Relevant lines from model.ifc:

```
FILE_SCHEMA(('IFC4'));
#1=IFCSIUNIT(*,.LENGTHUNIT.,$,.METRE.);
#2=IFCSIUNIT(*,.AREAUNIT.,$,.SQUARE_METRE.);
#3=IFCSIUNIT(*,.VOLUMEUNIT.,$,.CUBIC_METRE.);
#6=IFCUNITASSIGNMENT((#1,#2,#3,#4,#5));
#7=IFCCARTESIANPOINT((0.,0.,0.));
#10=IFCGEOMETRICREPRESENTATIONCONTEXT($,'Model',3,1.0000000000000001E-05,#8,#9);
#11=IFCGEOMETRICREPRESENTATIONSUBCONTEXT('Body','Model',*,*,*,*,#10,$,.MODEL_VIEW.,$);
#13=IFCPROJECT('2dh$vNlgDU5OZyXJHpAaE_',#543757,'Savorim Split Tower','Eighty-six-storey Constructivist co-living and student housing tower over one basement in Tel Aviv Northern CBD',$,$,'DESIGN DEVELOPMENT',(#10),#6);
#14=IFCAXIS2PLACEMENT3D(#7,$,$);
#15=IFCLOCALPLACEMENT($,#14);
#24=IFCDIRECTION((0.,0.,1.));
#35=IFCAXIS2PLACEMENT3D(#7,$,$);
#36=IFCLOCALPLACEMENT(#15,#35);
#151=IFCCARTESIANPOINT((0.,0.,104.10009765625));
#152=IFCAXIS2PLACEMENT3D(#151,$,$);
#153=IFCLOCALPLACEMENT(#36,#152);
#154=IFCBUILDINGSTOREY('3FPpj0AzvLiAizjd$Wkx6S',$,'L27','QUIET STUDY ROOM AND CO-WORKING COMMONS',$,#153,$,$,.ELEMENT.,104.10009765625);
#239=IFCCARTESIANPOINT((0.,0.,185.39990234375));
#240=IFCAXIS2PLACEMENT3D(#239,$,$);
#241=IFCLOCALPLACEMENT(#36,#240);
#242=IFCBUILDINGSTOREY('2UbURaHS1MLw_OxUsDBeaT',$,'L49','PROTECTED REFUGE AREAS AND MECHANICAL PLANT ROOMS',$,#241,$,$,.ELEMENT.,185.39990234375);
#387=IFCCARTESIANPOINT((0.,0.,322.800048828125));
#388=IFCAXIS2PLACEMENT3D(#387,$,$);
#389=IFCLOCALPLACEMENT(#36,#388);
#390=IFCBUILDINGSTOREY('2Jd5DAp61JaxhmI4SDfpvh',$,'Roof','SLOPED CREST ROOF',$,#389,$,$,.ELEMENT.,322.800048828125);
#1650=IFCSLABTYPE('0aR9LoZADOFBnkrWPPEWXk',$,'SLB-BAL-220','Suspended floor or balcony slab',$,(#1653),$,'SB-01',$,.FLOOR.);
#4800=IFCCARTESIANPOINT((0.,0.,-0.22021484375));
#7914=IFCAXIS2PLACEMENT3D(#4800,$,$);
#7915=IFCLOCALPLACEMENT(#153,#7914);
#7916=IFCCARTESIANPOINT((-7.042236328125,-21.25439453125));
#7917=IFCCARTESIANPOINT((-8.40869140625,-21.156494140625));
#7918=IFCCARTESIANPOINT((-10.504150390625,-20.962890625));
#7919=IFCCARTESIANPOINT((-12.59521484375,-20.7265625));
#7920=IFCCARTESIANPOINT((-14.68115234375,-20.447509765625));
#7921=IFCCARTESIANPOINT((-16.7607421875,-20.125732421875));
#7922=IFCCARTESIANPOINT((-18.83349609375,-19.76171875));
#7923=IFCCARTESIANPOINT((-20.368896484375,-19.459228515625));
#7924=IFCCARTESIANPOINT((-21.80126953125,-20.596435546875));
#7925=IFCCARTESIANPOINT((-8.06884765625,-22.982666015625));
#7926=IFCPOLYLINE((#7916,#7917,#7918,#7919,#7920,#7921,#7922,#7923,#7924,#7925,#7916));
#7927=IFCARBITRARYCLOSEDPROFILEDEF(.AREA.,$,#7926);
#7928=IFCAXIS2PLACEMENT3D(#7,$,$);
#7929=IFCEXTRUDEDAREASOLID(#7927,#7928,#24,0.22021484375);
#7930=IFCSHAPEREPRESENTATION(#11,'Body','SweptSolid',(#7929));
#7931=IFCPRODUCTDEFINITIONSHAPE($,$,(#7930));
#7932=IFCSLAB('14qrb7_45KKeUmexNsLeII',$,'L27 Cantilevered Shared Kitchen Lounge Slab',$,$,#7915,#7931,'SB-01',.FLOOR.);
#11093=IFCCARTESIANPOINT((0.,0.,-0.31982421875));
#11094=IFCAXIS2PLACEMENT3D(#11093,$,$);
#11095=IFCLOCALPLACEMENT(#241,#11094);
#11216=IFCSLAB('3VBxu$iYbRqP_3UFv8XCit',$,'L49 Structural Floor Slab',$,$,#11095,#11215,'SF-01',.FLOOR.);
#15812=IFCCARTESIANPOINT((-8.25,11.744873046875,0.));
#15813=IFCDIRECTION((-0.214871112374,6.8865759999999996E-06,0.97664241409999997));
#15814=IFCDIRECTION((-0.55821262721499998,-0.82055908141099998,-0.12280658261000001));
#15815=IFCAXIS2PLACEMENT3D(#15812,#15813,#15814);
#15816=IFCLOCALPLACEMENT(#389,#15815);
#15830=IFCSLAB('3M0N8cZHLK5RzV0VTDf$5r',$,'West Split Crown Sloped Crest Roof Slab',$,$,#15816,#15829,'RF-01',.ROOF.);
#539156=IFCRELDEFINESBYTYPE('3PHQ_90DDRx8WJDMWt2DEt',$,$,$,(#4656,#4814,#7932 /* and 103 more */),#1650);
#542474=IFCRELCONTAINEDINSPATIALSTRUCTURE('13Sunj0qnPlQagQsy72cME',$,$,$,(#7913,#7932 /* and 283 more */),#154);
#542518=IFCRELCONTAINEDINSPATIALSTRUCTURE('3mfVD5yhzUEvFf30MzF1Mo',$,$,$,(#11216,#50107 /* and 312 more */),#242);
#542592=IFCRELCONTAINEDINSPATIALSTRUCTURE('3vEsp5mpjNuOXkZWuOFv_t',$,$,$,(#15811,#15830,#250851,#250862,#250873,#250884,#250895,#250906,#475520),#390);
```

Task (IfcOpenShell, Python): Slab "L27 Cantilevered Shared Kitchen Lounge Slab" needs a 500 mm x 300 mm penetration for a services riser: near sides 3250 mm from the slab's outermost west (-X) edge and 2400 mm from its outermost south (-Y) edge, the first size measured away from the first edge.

```python
import numpy as np
import ifcopenshell
import ifcopenshell.api.feature
import ifcopenshell.api.geometry
import ifcopenshell.api.root
import ifcopenshell.geom
import ifcopenshell.util.placement
import ifcopenshell.util.representation
import ifcopenshell.util.shape
import ifcopenshell.util.unit

model = ifcopenshell.open("model.ifc")
unit_scale = ifcopenshell.util.unit.calculate_unit_scale(model)
settings = ifcopenshell.geom.settings()


def volume(element):
    """Net volume in cubic metres, openings subtracted."""
    shape = ifcopenshell.geom.create_shape(settings, element)
    return ifcopenshell.util.shape.get_volume(shape.geometry)


slab = model.by_id(7932)
before = volume(slab)

# Extent in the slab's own axes, in metres. The edges named are its -X and -Y sides.
slab_shape = ifcopenshell.geom.create_shape(settings, slab)
vertices = ifcopenshell.util.shape.get_vertices(slab_shape.geometry)
x_min, y_min, bottom = vertices.min(axis=0)
top = vertices[:, 2].max()

opening = ifcopenshell.api.root.create_entity(model, ifc_class="IfcOpeningElement", name="Services riser opening", predefined_type="OPENING")
context = ifcopenshell.util.representation.get_context(model, "Model", "Body", "MODEL_VIEW")
width, depth = 0.5, 0.3
outline = [(0.0, 0.0), (width, 0.0), (width, depth), (0.0, depth), (0.0, 0.0)]
# Overshoot both faces by 50 mm so the cut is clean.
shape = ifcopenshell.api.geometry.add_slab_representation(
    model, context=context, depth=top - bottom + 0.1, polyline=outline
)
ifcopenshell.api.geometry.assign_representation(model, product=opening, representation=shape)

matrix = ifcopenshell.util.placement.get_local_placement(slab.ObjectPlacement)
matrix[:, 3] = matrix @ np.append(np.array([x_min + 3.25, y_min + 2.4, bottom - 0.05]) / unit_scale, 1.0)
ifcopenshell.api.geometry.edit_object_placement(model, product=opening, matrix=matrix, is_si=False)
ifcopenshell.api.feature.add_feature(model, feature=opening, element=slab)

after = volume(slab)

print(f"slab volume {before:.3f} -> {after:.3f} m3")

model.write("model_edited.ifc")
```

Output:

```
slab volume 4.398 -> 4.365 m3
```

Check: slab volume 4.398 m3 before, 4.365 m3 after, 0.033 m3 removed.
